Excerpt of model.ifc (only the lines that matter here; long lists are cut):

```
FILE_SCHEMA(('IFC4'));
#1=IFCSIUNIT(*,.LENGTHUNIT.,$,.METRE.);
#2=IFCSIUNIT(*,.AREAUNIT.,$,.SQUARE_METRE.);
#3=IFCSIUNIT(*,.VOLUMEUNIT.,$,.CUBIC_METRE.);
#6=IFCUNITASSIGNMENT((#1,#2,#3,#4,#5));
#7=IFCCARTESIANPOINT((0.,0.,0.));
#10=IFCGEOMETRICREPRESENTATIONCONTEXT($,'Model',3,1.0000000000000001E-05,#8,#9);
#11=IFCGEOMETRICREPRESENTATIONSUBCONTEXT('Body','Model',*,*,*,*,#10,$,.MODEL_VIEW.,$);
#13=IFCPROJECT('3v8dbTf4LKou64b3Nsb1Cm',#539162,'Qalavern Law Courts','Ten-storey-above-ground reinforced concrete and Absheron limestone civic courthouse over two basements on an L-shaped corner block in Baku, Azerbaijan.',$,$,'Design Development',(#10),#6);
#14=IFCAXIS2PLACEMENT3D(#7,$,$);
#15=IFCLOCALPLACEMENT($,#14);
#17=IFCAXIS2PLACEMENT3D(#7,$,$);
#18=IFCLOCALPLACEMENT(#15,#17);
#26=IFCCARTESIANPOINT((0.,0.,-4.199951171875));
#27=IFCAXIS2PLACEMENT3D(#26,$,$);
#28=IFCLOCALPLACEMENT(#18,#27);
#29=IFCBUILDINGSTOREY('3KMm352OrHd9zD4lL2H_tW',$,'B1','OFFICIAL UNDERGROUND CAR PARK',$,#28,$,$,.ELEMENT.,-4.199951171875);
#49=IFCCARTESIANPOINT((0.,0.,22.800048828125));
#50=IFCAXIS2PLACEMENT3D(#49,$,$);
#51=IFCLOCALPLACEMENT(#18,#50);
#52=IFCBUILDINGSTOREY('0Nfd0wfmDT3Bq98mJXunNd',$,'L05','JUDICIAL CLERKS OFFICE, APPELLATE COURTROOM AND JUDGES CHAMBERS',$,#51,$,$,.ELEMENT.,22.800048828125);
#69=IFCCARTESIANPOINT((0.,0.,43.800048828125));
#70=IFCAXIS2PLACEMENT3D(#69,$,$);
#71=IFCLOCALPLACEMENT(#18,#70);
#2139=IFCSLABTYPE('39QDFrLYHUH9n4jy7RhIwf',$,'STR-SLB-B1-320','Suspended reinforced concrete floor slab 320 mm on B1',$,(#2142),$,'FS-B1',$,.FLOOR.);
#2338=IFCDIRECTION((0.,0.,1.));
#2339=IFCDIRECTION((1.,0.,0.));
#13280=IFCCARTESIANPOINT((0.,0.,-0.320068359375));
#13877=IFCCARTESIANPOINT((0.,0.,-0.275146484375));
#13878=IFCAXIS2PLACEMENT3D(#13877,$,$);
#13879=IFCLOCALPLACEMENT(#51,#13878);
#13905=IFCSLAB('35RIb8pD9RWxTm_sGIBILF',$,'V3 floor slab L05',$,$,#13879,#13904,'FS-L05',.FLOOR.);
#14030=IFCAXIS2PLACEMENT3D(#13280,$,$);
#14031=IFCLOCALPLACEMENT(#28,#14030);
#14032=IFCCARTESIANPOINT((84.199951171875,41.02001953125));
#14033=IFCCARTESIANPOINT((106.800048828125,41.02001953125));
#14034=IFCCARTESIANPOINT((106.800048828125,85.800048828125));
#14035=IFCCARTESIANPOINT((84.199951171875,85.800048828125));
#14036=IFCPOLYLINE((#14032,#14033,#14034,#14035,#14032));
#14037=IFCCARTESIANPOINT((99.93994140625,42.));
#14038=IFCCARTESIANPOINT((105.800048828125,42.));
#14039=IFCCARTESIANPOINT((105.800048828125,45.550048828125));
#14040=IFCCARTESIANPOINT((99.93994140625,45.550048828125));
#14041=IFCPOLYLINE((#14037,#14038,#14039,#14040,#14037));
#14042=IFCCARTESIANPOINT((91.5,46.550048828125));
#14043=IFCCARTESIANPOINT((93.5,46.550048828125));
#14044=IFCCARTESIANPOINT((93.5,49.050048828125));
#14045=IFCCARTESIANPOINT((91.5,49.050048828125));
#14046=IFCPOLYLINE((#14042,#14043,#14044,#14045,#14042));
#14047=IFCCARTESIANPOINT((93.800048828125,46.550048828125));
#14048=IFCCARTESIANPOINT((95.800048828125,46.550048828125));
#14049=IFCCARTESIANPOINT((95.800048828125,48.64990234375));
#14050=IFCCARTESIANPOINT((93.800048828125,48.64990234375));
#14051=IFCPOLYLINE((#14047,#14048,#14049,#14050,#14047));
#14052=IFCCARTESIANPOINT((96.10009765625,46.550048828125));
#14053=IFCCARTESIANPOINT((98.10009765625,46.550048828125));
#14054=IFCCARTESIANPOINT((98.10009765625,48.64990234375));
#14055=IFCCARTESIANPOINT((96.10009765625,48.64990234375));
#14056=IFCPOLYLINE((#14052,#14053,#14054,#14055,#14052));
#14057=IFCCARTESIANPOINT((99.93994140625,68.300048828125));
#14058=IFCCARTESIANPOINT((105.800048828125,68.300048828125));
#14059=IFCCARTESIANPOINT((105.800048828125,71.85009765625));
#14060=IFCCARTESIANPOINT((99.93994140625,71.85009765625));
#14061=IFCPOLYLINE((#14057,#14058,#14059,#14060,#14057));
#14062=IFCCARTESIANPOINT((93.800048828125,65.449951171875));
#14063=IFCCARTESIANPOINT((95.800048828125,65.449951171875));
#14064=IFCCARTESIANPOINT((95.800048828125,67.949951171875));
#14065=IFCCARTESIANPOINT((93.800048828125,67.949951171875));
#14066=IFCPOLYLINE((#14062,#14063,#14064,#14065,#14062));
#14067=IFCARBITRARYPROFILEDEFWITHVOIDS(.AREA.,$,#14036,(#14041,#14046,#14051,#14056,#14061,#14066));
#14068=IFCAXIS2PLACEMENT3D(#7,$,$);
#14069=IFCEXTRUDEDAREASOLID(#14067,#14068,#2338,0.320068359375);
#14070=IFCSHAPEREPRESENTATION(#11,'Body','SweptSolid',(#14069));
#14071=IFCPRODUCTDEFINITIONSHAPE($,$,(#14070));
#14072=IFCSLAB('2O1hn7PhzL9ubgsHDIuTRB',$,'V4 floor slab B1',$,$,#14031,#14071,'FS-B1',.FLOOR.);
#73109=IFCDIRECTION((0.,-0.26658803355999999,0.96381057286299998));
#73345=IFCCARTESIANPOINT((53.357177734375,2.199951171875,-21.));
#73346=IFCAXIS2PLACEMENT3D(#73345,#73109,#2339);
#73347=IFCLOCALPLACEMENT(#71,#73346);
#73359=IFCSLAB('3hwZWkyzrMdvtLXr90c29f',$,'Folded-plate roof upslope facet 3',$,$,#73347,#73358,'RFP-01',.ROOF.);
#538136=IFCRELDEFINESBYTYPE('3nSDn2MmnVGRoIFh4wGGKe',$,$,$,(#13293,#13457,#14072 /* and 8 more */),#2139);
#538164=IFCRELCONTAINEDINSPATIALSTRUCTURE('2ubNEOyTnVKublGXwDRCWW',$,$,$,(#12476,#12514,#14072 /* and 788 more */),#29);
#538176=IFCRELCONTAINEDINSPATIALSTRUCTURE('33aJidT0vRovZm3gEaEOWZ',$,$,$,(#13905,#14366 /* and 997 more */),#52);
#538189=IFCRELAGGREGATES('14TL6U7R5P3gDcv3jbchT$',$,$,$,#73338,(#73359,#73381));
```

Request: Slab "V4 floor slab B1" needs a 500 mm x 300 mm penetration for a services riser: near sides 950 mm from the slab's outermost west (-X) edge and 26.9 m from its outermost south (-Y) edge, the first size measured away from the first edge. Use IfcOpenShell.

```python
import numpy as np
import ifcopenshell
import ifcopenshell.api.feature
import ifcopenshell.api.geometry
import ifcopenshell.api.root
import ifcopenshell.geom
import ifcopenshell.util.placement
import ifcopenshell.util.representation
import ifcopenshell.util.shape
import ifcopenshell.util.unit

model = ifcopenshell.open("model.ifc")
unit_scale = ifcopenshell.util.unit.calculate_unit_scale(model)
settings = ifcopenshell.geom.settings()


def volume(element):
    """Net volume in cubic metres, openings subtracted."""
    shape = ifcopenshell.geom.create_shape(settings, element)
    return ifcopenshell.util.shape.get_volume(shape.geometry)


slab = model.by_guid("2O1hn7PhzL9ubgsHDIuTRB")
before = volume(slab)

# Extent in the slab's own axes, in metres. The edges named are its -X and -Y sides.
slab_shape = ifcopenshell.geom.create_shape(settings, slab)
vertices = ifcopenshell.util.shape.get_vertices(slab_shape.geometry)
x_min, y_min, bottom = vertices.min(axis=0)
top = vertices[:, 2].max()

opening = ifcopenshell.api.root.create_entity(model, ifc_class="IfcOpeningElement", name="Services riser opening", predefined_type="OPENING")
context = ifcopenshell.util.representation.get_context(model, "Model", "Body", "MODEL_VIEW")
width, depth = 0.5, 0.3
outline = [(0.0, 0.0), (width, 0.0), (width, depth), (0.0, depth), (0.0, 0.0)]
# Overshoot both faces by 50 mm so the cut is clean.
shape = ifcopenshell.api.geometry.add_slab_representation(
    model, context=context, depth=top - bottom + 0.1, polyline=outline
)
ifcopenshell.api.geometry.assign_representation(model, product=opening, representation=shape)

matrix = ifcopenshell.util.placement.get_local_placement(slab.ObjectPlacement)
matrix[:, 3] = matrix @ np.append(np.array([x_min + 0.95, y_min + 26.9, bottom - 0.05]) / unit_scale, 1.0)
ifcopenshell.api.geometry.edit_object_placement(model, product=opening, matrix=matrix, is_si=False)
ifcopenshell.api.feature.add_feature(model, feature=opening, element=slab)

after = volume(slab)

print(f"slab volume {before:.3f} -> {after:.3f} m3")

model.write("model_edited.ifc")
```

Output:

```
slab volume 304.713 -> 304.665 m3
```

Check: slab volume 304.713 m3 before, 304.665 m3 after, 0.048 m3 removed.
